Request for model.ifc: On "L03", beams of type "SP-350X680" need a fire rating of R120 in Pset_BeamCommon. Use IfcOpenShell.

First a look at what the model holds.

```python
import ifcopenshell
import ifcopenshell.util.element

model = ifcopenshell.open("model.ifc")
print(model.schema)
storey = next(s for s in model.by_type("IfcBuildingStorey") if s.Name == "L03")
beams = [e for e in ifcopenshell.util.element.get_decomposition(storey) if e.is_a("IfcBeam")]
seen = {}
for e in beams:
    element_type = ifcopenshell.util.element.get_type(e)
    key = (element_type.Name if element_type != e and element_type else None, ifcopenshell.util.element.get_pset(e, "Pset_BeamCommon", "FireRating"))
    seen[key] = seen.get(key, 0) + 1
for (name, value), count in sorted(seen.items(), key=str):
    print(count, "x", name, "|", value)
```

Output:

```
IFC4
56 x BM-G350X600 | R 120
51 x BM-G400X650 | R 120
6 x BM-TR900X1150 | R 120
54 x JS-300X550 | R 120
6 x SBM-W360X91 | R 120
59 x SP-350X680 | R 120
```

```python
import ifcopenshell
import ifcopenshell.api.pset
import ifcopenshell.util.element

model = ifcopenshell.open("model.ifc")

storey = next(s for s in model.by_type("IfcBuildingStorey") if s.Name == "L03")
beams = [e for e in ifcopenshell.util.element.get_decomposition(storey) if e.is_a("IfcBeam")]

count = 0
for e in beams:
    element_type = ifcopenshell.util.element.get_type(e)
    if element_type in (None, e) or element_type.Name != "SP-350X680":
        continue
    # add_pset returns the element's existing set when there is one.
    pset = ifcopenshell.api.pset.add_pset(model, product=e, name="Pset_BeamCommon")
    ifcopenshell.api.pset.edit_pset(model, pset=pset, properties={"FireRating": "R120"})
    count += 1

print(count, "beams updated")

model.write("model_v2.ifc")
```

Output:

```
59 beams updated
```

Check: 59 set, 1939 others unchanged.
